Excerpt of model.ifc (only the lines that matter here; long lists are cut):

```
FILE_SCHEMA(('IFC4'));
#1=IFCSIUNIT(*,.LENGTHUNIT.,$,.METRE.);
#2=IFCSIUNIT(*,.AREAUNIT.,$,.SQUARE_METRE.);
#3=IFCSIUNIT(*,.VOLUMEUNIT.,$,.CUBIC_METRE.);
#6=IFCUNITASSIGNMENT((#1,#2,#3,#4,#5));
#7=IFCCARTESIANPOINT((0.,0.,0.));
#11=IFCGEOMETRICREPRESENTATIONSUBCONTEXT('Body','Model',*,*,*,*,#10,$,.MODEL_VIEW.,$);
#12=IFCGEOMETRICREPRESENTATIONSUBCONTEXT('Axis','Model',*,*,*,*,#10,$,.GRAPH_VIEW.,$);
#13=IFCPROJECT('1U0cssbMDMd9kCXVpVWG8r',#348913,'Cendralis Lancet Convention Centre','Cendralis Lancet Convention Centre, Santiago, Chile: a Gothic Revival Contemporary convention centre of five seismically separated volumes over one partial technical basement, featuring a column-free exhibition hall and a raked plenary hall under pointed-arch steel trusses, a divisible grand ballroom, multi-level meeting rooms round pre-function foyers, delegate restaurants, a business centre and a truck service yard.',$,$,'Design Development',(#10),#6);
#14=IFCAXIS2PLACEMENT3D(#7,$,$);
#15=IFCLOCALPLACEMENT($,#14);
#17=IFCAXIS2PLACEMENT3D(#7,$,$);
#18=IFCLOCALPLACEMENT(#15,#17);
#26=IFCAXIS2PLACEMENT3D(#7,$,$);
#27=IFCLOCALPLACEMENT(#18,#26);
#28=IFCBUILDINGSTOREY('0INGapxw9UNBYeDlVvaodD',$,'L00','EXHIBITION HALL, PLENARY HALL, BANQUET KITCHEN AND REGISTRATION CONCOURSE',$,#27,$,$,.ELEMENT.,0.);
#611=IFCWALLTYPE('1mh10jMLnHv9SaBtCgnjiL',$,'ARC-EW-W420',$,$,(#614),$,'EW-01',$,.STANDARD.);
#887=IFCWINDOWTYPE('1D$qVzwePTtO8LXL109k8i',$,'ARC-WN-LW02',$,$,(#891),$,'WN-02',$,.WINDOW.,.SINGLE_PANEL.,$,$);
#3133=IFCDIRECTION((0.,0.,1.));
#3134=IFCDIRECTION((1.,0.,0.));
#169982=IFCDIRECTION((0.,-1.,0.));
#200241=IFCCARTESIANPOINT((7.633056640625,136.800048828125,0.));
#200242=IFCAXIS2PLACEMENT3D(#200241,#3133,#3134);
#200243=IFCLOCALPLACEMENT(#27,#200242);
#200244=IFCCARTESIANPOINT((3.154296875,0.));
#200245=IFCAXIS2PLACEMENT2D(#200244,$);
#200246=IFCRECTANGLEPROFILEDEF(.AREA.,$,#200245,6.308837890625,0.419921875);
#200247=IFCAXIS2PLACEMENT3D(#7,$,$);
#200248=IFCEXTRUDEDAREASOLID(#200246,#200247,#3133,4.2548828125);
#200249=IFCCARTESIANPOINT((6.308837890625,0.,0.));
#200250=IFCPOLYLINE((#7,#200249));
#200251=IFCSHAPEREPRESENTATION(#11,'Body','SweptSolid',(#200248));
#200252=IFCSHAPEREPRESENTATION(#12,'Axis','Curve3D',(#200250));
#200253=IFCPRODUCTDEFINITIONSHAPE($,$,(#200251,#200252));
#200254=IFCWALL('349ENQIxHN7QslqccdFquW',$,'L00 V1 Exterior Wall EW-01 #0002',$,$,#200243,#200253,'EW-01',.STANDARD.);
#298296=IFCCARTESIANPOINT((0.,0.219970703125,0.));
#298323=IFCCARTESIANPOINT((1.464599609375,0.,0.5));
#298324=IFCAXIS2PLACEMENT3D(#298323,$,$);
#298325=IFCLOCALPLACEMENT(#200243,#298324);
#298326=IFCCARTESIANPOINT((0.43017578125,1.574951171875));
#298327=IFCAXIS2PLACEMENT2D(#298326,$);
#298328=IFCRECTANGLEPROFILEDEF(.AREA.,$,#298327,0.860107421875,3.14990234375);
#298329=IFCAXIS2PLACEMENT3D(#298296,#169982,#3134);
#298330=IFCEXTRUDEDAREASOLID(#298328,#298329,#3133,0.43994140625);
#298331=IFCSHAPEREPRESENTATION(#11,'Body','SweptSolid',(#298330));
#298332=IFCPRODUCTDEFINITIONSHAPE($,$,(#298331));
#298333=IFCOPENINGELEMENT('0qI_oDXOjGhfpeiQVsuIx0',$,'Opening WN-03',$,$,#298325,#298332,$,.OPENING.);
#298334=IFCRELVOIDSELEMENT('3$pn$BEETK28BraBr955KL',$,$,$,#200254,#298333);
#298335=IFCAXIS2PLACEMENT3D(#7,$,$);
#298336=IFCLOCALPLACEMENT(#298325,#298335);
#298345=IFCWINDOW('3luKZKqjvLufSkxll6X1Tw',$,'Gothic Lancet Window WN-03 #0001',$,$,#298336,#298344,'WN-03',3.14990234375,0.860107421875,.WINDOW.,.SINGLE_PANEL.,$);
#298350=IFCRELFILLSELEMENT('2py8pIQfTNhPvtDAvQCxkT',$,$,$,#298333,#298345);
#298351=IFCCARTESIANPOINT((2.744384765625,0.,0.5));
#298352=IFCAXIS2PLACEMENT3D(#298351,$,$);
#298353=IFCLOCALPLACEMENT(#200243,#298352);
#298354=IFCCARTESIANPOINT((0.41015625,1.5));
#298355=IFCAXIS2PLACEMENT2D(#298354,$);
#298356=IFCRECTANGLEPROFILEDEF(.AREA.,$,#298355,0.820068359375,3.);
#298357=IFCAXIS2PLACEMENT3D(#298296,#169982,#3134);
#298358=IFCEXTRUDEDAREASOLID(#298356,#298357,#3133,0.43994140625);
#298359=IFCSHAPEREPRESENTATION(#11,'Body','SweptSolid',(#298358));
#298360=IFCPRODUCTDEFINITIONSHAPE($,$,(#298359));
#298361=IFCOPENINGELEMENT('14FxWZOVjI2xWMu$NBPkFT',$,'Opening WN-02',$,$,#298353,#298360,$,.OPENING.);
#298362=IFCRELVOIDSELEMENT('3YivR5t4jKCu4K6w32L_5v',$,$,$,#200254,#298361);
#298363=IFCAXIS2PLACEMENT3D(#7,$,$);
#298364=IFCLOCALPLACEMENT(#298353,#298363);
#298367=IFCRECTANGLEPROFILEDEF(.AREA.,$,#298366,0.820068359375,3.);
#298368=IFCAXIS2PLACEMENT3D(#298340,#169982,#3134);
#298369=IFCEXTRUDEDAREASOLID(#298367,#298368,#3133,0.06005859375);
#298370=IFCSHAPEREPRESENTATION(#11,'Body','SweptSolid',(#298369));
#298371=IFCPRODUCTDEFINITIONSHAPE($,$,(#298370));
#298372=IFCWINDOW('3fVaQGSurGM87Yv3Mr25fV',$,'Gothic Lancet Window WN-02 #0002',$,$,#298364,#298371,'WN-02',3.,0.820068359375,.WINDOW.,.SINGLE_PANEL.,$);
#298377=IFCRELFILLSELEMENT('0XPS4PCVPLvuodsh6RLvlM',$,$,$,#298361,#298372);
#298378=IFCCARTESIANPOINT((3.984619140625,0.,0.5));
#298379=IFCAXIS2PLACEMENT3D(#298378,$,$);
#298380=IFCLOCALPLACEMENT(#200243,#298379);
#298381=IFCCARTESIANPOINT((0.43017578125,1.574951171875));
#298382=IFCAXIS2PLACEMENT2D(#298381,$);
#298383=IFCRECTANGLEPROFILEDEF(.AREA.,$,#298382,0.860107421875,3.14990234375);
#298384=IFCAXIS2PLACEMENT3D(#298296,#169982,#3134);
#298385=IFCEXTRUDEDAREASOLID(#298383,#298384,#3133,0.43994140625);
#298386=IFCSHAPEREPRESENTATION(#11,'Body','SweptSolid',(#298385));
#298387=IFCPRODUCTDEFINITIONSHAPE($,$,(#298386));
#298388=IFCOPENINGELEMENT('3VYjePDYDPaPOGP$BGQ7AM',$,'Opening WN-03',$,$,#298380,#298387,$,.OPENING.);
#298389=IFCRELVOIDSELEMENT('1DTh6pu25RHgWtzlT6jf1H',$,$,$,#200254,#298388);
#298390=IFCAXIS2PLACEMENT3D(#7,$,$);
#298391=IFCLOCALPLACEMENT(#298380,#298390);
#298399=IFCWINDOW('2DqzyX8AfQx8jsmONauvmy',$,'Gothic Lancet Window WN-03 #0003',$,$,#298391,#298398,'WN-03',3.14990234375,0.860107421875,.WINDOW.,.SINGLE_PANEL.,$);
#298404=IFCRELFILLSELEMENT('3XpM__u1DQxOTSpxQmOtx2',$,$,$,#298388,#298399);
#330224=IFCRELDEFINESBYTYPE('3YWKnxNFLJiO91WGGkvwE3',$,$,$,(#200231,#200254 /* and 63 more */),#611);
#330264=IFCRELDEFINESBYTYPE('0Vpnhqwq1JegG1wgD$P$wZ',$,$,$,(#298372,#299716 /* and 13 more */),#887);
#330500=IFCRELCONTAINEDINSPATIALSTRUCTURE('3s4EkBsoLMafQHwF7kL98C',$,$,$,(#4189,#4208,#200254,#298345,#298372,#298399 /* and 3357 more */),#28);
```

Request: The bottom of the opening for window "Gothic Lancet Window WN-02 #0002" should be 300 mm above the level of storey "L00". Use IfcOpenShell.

```python
import numpy as np
import ifcopenshell
import ifcopenshell.api.geometry
import ifcopenshell.geom
import ifcopenshell.util.element
import ifcopenshell.util.placement
import ifcopenshell.util.shape
import ifcopenshell.util.unit

model = ifcopenshell.open("model.ifc")
unit_scale = ifcopenshell.util.unit.calculate_unit_scale(model)

window = model.by_id(298372)
opening = window.FillsVoids[0].RelatingOpeningElement
storey = ifcopenshell.util.element.get_container(window, ifc_class="IfcBuildingStorey")
level = ifcopenshell.util.placement.get_local_placement(storey.ObjectPlacement)[2, 3]

# The opening's origin need not be at the sill, so measure its lowest point.
shape = ifcopenshell.geom.create_shape(ifcopenshell.geom.settings(), opening)
bottom = ifcopenshell.util.shape.get_shape_bottom_elevation(shape, shape.geometry) / unit_scale
dz = level + 0.3 / unit_scale - bottom

shift = np.array([0.0, 0.0, dz])
# The window is placed relative to its opening, so it follows when the opening moves.
matrix = ifcopenshell.util.placement.get_local_placement(opening.ObjectPlacement)
matrix[:3, 3] += shift
ifcopenshell.api.geometry.edit_object_placement(
    model, product=opening, matrix=matrix, is_si=False, should_transform_children=True
)

print(f"moved by {dz * unit_scale:+.3f} m")

model.write("model-out.ifc")
```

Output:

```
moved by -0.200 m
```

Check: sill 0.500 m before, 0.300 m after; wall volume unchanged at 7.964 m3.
